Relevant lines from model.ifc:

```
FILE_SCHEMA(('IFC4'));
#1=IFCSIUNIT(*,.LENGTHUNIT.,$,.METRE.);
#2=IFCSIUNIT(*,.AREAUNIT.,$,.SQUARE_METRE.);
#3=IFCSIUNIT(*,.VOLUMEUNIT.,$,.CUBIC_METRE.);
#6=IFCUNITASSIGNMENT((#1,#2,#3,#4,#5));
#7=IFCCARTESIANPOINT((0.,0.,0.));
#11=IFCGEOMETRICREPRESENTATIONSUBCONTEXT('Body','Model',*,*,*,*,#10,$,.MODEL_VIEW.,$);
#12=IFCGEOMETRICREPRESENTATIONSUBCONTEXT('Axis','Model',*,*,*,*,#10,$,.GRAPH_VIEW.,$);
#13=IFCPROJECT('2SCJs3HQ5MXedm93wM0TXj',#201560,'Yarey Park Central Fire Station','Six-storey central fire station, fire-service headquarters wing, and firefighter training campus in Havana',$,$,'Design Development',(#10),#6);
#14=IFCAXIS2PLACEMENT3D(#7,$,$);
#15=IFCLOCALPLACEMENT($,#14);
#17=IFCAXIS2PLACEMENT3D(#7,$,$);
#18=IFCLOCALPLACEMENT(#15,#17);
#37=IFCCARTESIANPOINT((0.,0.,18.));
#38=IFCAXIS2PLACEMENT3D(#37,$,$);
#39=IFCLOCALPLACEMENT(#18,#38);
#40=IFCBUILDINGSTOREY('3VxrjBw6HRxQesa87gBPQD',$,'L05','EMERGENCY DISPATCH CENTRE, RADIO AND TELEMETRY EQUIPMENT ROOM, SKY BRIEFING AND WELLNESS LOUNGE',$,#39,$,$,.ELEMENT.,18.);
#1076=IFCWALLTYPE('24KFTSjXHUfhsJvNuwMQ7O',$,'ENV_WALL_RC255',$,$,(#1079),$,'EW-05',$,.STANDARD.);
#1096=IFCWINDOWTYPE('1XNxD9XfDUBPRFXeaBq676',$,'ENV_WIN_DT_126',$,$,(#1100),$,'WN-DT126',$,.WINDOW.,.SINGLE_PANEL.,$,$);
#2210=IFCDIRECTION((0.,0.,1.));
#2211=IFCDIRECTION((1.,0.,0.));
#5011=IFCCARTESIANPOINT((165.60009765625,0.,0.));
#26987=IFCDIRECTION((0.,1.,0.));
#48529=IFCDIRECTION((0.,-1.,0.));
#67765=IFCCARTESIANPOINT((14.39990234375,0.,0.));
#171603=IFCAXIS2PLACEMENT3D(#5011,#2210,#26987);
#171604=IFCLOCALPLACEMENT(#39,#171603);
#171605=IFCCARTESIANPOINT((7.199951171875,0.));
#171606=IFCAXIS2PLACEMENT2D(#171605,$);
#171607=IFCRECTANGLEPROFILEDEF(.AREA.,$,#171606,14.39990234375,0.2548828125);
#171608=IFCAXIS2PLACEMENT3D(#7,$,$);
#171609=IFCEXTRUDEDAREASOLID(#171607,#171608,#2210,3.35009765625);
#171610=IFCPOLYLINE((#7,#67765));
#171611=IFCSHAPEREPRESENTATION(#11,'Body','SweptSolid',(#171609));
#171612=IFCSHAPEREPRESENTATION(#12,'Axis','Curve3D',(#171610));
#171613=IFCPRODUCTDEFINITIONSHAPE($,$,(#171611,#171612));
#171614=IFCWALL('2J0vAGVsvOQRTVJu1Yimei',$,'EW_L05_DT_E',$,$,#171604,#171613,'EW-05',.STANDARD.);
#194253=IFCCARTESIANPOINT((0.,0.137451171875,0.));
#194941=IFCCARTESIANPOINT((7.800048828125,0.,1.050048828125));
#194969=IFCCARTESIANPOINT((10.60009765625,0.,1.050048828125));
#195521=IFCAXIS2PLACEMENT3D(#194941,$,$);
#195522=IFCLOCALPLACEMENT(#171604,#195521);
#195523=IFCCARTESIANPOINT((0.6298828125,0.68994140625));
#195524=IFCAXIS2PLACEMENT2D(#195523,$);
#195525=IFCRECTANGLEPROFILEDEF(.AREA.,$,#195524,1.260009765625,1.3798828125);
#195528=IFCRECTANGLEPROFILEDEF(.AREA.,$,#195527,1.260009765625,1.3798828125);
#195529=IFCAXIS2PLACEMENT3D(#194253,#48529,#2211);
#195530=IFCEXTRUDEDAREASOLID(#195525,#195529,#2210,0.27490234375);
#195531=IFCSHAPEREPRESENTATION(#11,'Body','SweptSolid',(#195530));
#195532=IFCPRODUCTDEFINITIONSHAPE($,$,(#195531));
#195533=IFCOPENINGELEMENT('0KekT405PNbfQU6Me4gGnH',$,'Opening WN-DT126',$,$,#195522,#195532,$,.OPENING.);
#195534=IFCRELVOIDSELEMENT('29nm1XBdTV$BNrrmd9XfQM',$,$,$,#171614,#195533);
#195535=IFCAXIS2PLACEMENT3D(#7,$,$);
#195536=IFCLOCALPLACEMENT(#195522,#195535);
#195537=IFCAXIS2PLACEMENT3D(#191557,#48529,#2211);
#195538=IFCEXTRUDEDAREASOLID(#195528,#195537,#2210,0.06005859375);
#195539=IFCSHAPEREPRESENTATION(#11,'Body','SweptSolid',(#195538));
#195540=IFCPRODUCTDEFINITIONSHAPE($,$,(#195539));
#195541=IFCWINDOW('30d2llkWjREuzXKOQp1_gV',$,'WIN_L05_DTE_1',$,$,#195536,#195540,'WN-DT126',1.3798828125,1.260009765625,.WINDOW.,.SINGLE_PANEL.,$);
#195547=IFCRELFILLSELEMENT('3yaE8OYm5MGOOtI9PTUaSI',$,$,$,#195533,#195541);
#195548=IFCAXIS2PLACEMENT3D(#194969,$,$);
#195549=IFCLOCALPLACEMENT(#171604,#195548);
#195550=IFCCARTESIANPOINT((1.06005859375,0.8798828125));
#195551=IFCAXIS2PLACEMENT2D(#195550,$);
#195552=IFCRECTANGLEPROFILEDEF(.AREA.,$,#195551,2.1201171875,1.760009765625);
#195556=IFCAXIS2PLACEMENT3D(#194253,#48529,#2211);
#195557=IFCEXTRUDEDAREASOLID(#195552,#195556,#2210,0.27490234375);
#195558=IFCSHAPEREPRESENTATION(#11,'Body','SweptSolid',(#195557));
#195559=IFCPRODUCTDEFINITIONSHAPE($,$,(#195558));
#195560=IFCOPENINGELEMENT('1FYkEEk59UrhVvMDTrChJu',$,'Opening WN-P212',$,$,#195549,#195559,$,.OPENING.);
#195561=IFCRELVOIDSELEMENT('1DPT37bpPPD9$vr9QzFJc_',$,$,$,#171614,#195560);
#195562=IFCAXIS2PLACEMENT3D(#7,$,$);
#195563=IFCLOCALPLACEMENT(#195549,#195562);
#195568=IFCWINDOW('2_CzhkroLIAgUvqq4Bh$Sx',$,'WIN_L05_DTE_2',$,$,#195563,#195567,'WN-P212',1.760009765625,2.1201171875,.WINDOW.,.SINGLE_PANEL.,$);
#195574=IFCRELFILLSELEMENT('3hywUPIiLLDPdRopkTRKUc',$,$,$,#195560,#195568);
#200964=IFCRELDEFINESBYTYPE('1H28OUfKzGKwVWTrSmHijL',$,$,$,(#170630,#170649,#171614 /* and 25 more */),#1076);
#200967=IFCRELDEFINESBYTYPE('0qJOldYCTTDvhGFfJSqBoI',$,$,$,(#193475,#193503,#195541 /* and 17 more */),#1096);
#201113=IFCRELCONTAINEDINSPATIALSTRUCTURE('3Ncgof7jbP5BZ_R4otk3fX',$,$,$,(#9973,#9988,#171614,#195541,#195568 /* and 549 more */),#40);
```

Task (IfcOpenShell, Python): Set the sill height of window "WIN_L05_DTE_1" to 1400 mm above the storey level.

```python
import numpy as np
import ifcopenshell
import ifcopenshell.api.geometry
import ifcopenshell.geom
import ifcopenshell.util.element
import ifcopenshell.util.placement
import ifcopenshell.util.shape
import ifcopenshell.util.unit

model = ifcopenshell.open("model.ifc")
unit_scale = ifcopenshell.util.unit.calculate_unit_scale(model)

window = model.by_id(195541)
opening = window.FillsVoids[0].RelatingOpeningElement
storey = ifcopenshell.util.element.get_container(window, ifc_class="IfcBuildingStorey")
level = ifcopenshell.util.placement.get_local_placement(storey.ObjectPlacement)[2, 3]

# The opening's origin need not be at the sill, so measure its lowest point.
shape = ifcopenshell.geom.create_shape(ifcopenshell.geom.settings(), opening)
bottom = ifcopenshell.util.shape.get_shape_bottom_elevation(shape, shape.geometry) / unit_scale
dz = level + 1.4 - bottom

shift = np.array([0.0, 0.0, dz])
# The window is placed relative to its opening, so it follows when the opening moves.
matrix = ifcopenshell.util.placement.get_local_placement(opening.ObjectPlacement)
matrix[:3, 3] += shift
ifcopenshell.api.geometry.edit_object_placement(
    model, product=opening, matrix=matrix, is_si=False, should_transform_children=True
)

print(f"moved by {dz * unit_scale:+.3f} m")

model.write("model_rev.ifc")
```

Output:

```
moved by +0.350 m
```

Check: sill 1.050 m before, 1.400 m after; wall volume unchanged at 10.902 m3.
